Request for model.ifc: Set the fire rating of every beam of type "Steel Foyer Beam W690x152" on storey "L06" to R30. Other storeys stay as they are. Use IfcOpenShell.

First a look at what the model holds.

```python
import ifcopenshell
import ifcopenshell.util.element

model = ifcopenshell.open("model.ifc")
print(model.schema)
storey = next(s for s in model.by_type("IfcBuildingStorey") if s.Name == "L06")
beams = [e for e in ifcopenshell.util.element.get_decomposition(storey) if e.is_a("IfcBeam")]
seen = {}
for e in beams:
    element_type = ifcopenshell.util.element.get_type(e)
    key = (element_type.Name if element_type != e and element_type else None, ifcopenshell.util.element.get_pset(e, "Pset_BeamCommon", "FireRating"))
    seen[key] = seen.get(key, 0) + 1
for (name, value), count in sorted(seen.items(), key=str):
    print(count, "x", name, "|", value)
```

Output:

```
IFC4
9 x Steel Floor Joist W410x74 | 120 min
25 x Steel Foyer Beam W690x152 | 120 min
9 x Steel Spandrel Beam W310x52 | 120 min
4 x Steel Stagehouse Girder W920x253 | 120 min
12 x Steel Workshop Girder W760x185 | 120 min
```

```python
import ifcopenshell
import ifcopenshell.api.pset
import ifcopenshell.util.element

model = ifcopenshell.open("model.ifc")

storey = next(s for s in model.by_type("IfcBuildingStorey") if s.Name == "L06")
beams = [e for e in ifcopenshell.util.element.get_decomposition(storey) if e.is_a("IfcBeam")]

count = 0
for e in beams:
    element_type = ifcopenshell.util.element.get_type(e)
    if element_type in (None, e) or element_type.Name != "Steel Foyer Beam W690x152":
        continue
    # add_pset returns the element's existing set when there is one.
    pset = ifcopenshell.api.pset.add_pset(model, product=e, name="Pset_BeamCommon")
    ifcopenshell.api.pset.edit_pset(model, pset=pset, properties={"FireRating": "R30"})
    count += 1

print(count, "beams updated")

model.write("model_rev.ifc")
```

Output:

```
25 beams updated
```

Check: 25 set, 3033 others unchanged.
